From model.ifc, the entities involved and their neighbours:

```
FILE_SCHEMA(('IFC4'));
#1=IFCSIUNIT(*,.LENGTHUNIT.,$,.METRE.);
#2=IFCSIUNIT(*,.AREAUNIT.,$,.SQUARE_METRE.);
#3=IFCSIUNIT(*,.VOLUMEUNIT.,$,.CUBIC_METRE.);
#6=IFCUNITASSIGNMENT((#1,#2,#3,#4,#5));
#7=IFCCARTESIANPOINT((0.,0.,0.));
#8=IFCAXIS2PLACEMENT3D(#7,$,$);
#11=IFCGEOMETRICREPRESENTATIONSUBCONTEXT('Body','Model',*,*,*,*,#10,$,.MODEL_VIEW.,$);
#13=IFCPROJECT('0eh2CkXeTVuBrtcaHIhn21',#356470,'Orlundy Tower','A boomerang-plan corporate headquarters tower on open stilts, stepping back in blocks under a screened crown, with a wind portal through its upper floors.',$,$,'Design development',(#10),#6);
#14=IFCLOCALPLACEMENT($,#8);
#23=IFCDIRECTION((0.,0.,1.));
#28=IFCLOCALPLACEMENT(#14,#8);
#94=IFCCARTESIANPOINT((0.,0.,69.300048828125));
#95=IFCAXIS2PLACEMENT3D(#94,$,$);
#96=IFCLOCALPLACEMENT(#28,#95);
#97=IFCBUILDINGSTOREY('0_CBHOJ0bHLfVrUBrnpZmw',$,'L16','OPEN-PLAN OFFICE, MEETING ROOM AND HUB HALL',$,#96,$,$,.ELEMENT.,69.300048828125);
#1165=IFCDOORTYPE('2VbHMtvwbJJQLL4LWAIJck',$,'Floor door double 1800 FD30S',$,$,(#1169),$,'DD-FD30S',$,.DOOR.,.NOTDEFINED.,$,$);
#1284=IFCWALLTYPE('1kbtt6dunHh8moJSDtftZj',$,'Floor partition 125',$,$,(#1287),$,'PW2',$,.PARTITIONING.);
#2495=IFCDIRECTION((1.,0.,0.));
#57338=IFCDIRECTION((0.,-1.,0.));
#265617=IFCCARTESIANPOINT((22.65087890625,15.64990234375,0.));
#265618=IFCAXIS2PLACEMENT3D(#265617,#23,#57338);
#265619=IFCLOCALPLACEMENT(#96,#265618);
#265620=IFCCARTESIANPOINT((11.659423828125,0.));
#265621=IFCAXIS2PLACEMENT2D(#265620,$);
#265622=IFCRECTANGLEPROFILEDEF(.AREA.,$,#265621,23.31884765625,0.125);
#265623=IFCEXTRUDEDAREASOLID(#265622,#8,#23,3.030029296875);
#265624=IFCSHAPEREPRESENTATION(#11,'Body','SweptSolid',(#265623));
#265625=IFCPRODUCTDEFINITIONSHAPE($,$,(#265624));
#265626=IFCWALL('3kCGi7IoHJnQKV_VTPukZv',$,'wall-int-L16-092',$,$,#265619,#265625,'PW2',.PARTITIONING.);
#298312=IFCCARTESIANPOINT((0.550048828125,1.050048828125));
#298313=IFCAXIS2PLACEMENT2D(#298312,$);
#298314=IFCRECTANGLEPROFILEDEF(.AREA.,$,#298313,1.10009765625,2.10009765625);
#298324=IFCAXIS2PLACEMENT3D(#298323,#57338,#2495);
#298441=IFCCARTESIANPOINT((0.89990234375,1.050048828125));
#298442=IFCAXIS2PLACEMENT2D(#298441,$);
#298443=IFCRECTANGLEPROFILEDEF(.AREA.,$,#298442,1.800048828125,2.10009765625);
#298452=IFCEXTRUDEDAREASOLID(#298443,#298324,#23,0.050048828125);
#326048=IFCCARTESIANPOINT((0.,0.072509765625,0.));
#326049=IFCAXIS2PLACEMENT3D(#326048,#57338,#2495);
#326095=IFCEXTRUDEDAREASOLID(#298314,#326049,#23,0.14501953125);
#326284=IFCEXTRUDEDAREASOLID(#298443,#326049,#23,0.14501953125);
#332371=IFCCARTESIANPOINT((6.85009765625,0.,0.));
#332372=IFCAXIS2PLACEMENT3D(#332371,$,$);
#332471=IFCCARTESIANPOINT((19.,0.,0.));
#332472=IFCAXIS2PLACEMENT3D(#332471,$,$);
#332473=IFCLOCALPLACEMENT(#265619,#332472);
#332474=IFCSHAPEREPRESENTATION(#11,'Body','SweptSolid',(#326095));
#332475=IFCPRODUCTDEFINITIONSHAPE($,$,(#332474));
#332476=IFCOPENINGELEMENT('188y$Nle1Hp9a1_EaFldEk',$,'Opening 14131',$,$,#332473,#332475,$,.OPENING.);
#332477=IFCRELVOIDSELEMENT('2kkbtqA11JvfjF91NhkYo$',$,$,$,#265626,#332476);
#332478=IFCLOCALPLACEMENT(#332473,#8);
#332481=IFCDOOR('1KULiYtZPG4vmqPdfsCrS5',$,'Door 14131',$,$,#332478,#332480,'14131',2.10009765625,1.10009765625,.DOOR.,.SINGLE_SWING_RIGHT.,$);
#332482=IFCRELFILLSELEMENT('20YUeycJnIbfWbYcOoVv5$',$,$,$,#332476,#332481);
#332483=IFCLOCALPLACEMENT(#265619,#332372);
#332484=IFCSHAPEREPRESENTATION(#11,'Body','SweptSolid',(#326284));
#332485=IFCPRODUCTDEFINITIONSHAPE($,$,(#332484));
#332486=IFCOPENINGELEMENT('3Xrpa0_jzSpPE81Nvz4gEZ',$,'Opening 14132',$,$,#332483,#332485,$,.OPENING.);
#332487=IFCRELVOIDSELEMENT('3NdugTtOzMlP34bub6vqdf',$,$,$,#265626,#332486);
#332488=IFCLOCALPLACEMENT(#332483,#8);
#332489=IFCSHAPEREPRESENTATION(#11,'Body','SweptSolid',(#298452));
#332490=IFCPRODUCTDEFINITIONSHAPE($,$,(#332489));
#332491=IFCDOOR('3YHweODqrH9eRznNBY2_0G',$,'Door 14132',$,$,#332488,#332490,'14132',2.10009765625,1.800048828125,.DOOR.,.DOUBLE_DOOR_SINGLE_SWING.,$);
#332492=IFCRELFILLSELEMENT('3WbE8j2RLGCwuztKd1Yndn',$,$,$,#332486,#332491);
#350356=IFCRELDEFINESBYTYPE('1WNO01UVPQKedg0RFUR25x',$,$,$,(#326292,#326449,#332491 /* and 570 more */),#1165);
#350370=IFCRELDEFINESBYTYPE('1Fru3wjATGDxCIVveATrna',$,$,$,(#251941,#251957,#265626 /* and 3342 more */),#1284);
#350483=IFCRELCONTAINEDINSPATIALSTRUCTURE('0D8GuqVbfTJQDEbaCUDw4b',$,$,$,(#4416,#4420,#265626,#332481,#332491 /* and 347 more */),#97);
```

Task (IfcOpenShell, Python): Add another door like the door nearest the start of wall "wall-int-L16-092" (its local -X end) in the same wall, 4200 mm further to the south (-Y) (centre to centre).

```python
import ifcopenshell
import ifcopenshell.api.feature
import ifcopenshell.api.geometry
import ifcopenshell.api.root
import ifcopenshell.geom
import ifcopenshell.util.element
import ifcopenshell.util.placement
import ifcopenshell.util.shape
import ifcopenshell.util.unit

model = ifcopenshell.open("model.ifc")
unit_scale = ifcopenshell.util.unit.calculate_unit_scale(model)
settings = ifcopenshell.geom.settings()


def volume(element):
    """Net volume in cubic metres, openings subtracted."""
    shape = ifcopenshell.geom.create_shape(settings, element)
    return ifcopenshell.util.shape.get_volume(shape.geometry)


door = model.by_guid("3YHweODqrH9eRznNBY2_0G")
opening = door.FillsVoids[0].RelatingOpeningElement
wall = opening.VoidsElements[0].RelatingBuildingElement
before = volume(wall)
shift = ifcopenshell.util.placement.get_local_placement(wall.ObjectPlacement)[:3, 0] * 4.2 / unit_scale

# copy_class copies the void relationship, type, container and properties, but no geometry.
new_opening = ifcopenshell.api.root.copy_class(model, product=opening)
new_opening.Representation = ifcopenshell.util.element.copy_deep(
    model, opening.Representation, exclude=["IfcGeometricRepresentationContext", "IfcRepresentationMap"]
)
new_door = ifcopenshell.api.root.copy_class(model, product=door)
new_door.Representation = ifcopenshell.util.element.copy_deep(
    model, door.Representation, exclude=["IfcGeometricRepresentationContext", "IfcRepresentationMap"]
)
new_door.Tag = None
ifcopenshell.api.feature.add_filling(model, opening=new_opening, element=new_door)

for old, new in ((opening, new_opening), (door, new_door)):
    matrix = ifcopenshell.util.placement.get_local_placement(old.ObjectPlacement)
    matrix[:3, 3] += shift
    ifcopenshell.api.geometry.edit_object_placement(model, product=new, matrix=matrix, is_si=False)

after = volume(wall)

print(f"wall volume {before:.3f} -> {after:.3f} m3")

model.write("model-out.ifc")
```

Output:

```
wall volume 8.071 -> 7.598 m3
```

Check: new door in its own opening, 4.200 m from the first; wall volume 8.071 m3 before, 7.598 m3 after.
